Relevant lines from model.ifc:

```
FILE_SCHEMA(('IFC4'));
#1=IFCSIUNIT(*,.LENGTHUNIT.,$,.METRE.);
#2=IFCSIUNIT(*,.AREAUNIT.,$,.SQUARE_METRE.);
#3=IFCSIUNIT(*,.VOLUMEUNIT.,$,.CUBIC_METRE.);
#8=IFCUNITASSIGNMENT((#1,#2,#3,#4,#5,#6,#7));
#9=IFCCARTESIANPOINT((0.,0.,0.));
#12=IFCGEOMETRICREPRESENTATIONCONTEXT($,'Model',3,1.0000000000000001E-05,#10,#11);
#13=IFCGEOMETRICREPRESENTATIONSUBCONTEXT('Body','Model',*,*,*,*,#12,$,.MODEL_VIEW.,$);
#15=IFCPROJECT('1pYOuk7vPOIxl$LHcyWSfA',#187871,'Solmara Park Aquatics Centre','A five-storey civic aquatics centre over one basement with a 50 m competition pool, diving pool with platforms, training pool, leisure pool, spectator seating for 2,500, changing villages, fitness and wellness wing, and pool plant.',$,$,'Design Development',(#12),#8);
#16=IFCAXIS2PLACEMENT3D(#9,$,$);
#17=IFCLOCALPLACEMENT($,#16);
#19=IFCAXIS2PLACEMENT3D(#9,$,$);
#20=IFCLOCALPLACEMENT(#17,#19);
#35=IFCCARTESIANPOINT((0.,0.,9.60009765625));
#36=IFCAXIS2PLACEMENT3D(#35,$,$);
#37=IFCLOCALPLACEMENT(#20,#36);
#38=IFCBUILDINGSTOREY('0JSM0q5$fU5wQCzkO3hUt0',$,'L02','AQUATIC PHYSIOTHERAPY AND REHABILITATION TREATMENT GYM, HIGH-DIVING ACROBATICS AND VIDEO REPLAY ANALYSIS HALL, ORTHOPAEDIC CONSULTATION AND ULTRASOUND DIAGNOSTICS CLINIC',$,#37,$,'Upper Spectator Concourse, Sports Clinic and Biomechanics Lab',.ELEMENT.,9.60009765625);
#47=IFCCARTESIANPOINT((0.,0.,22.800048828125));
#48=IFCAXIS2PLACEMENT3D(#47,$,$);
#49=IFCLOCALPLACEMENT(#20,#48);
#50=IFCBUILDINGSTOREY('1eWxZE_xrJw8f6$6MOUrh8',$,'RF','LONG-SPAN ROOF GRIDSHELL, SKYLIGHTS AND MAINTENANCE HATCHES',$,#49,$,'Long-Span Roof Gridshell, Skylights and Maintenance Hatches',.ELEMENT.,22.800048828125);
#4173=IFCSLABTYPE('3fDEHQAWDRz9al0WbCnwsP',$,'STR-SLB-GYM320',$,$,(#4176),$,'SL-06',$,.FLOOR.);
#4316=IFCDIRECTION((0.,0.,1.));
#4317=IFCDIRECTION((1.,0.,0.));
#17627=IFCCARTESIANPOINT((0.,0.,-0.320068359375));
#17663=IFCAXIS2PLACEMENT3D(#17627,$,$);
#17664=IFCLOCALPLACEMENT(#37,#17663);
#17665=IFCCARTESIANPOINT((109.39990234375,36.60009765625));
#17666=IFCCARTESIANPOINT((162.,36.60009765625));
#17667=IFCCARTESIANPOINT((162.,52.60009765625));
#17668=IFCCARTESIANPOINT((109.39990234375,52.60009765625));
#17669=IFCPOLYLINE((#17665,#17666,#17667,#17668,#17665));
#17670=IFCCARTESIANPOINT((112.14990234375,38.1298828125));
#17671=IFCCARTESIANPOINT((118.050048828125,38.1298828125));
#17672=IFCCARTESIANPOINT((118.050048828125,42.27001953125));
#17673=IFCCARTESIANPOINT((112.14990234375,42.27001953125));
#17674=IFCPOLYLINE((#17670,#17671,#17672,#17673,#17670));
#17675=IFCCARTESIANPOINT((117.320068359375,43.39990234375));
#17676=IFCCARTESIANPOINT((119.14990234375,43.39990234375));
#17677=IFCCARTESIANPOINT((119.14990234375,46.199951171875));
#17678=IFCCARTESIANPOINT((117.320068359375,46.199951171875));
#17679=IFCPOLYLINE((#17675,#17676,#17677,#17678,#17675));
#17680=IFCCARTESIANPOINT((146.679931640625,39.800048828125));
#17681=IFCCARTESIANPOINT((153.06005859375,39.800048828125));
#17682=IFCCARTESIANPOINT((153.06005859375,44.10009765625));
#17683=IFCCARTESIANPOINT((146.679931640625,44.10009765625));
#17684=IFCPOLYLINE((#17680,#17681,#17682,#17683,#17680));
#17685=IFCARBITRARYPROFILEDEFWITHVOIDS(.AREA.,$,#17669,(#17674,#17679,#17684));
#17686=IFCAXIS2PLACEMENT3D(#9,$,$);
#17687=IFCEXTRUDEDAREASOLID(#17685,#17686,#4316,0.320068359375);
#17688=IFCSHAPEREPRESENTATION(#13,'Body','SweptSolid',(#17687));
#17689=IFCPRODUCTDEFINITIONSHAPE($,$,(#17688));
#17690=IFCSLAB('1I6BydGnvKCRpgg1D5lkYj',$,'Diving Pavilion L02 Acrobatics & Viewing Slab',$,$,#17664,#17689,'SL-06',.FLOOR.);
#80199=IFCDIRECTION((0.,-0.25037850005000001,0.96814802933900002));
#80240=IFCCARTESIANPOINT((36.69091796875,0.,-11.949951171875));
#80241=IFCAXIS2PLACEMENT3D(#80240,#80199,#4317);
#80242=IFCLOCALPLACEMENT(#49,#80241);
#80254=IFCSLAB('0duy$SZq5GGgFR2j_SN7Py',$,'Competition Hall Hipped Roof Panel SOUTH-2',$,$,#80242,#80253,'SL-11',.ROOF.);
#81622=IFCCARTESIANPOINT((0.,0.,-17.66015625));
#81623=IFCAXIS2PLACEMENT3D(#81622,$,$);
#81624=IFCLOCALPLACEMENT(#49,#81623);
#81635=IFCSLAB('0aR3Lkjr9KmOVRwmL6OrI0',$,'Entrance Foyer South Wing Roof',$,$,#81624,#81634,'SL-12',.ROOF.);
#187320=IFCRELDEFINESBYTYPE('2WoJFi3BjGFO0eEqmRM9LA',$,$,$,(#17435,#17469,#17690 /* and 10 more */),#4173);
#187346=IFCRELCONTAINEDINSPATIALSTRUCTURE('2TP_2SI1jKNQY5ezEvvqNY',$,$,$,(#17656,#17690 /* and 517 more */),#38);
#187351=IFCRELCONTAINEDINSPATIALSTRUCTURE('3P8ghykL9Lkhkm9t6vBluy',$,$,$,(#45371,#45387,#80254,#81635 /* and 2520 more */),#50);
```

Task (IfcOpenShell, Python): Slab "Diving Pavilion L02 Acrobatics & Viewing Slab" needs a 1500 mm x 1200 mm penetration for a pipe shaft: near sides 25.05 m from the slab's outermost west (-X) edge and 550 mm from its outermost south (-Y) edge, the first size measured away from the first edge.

```python
import numpy as np
import ifcopenshell
import ifcopenshell.api.feature
import ifcopenshell.api.geometry
import ifcopenshell.api.root
import ifcopenshell.geom
import ifcopenshell.util.placement
import ifcopenshell.util.representation
import ifcopenshell.util.shape
import ifcopenshell.util.unit

model = ifcopenshell.open("model.ifc")
unit_scale = ifcopenshell.util.unit.calculate_unit_scale(model)
settings = ifcopenshell.geom.settings()


def volume(element):
    """Net volume in cubic metres, openings subtracted."""
    shape = ifcopenshell.geom.create_shape(settings, element)
    return ifcopenshell.util.shape.get_volume(shape.geometry)


slab = model.by_guid("1I6BydGnvKCRpgg1D5lkYj")
before = volume(slab)

# Extent in the slab's own axes, in metres. The edges named are its -X and -Y sides.
slab_shape = ifcopenshell.geom.create_shape(settings, slab)
vertices = ifcopenshell.util.shape.get_vertices(slab_shape.geometry)
x_min, y_min, bottom = vertices.min(axis=0)
top = vertices[:, 2].max()

opening = ifcopenshell.api.root.create_entity(model, ifc_class="IfcOpeningElement", name="Pipe shaft opening", predefined_type="OPENING")
context = ifcopenshell.util.representation.get_context(model, "Model", "Body", "MODEL_VIEW")
width, depth = 1.5, 1.2
outline = [(0.0, 0.0), (width, 0.0), (width, depth), (0.0, depth), (0.0, 0.0)]
# Overshoot both faces by 50 mm so the cut is clean.
shape = ifcopenshell.api.geometry.add_slab_representation(
    model, context=context, depth=top - bottom + 0.1, polyline=outline
)
ifcopenshell.api.geometry.assign_representation(model, product=opening, representation=shape)

matrix = ifcopenshell.util.placement.get_local_placement(slab.ObjectPlacement)
matrix[:, 3] = matrix @ np.append(np.array([x_min + 25.05, y_min + 0.55, bottom - 0.05]) / unit_scale, 1.0)
ifcopenshell.api.geometry.edit_object_placement(model, product=opening, matrix=matrix, is_si=False)
ifcopenshell.api.feature.add_feature(model, feature=opening, element=slab)

after = volume(slab)

print(f"slab volume {before:.3f} -> {after:.3f} m3")

model.write("model_updated.ifc")
```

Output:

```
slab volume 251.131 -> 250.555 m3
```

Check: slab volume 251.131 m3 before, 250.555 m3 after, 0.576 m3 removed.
